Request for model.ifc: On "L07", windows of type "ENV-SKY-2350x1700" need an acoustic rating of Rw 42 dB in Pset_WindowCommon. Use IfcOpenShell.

First a look at what the model holds.

```python
import ifcopenshell
import ifcopenshell.util.element

model = ifcopenshell.open("model.ifc")
print(model.schema)
storey = next(s for s in model.by_type("IfcBuildingStorey") if s.Name == "L07")
windows = [e for e in ifcopenshell.util.element.get_decomposition(storey) if e.is_a("IfcWindow")]
seen = {}
for e in windows:
    element_type = ifcopenshell.util.element.get_type(e)
    key = (element_type.Name if element_type != e and element_type else None, ifcopenshell.util.element.get_pset(e, "Pset_WindowCommon", "AcousticRating"))
    seen[key] = seen.get(key, 0) + 1
for (name, value), count in sorted(seen.items(), key=str):
    print(count, "x", name, "|", value)
```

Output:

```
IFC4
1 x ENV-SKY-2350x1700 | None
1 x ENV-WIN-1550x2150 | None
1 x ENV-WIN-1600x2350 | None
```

```python
import ifcopenshell
import ifcopenshell.api.pset
import ifcopenshell.util.element

model = ifcopenshell.open("model.ifc")

storey = next(s for s in model.by_type("IfcBuildingStorey") if s.Name == "L07")
windows = [e for e in ifcopenshell.util.element.get_decomposition(storey) if e.is_a("IfcWindow")]

count = 0
for e in windows:
    element_type = ifcopenshell.util.element.get_type(e)
    if element_type in (None, e) or element_type.Name != "ENV-SKY-2350x1700":
        continue
    # add_pset returns the element's existing set when there is one.
    pset = ifcopenshell.api.pset.add_pset(model, product=e, name="Pset_WindowCommon")
    ifcopenshell.api.pset.edit_pset(model, pset=pset, properties={"AcousticRating": "Rw 42 dB"})
    count += 1

print(count, "windows updated")

model.write("model_edited.ifc")
```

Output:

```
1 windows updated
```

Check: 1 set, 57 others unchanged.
